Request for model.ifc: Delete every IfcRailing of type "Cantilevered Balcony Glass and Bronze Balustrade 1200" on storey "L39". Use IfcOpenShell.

First a look at what the model holds.

```python
import ifcopenshell
import ifcopenshell.util.element

model = ifcopenshell.open("model.ifc")
print(model.schema)
storey = next(s for s in model.by_type("IfcBuildingStorey") if s.Name == "L39")
railings = [e for e in ifcopenshell.util.element.get_decomposition(storey) if e.is_a("IfcRailing")]
seen = {}
for e in railings:
    element_type = ifcopenshell.util.element.get_type(e)
    name = element_type.Name if element_type not in (None, e) else None
    seen[name] = seen.get(name, 0) + 1
for name, count in sorted(seen.items(), key=str):
    print(count, "x", name)
```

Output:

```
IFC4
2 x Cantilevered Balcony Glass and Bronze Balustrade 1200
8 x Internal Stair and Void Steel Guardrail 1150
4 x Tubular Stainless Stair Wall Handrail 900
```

```python
import ifcopenshell
import ifcopenshell.api.root
import ifcopenshell.util.element

model = ifcopenshell.open("model.ifc")

storey = next(s for s in model.by_type("IfcBuildingStorey") if s.Name == "L39")
railings = [e for e in ifcopenshell.util.element.get_decomposition(storey) if e.is_a("IfcRailing")]
targets = [e for e in railings if (t := ifcopenshell.util.element.get_type(e)) not in (None, e) and t.Name == "Cantilevered Balcony Glass and Bronze Balustrade 1200"]

for e in targets:
    ifcopenshell.api.root.remove_product(model, product=e)
print(len(targets), "removed")

model.write("model_rev.ifc")
```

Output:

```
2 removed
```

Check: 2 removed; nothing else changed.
